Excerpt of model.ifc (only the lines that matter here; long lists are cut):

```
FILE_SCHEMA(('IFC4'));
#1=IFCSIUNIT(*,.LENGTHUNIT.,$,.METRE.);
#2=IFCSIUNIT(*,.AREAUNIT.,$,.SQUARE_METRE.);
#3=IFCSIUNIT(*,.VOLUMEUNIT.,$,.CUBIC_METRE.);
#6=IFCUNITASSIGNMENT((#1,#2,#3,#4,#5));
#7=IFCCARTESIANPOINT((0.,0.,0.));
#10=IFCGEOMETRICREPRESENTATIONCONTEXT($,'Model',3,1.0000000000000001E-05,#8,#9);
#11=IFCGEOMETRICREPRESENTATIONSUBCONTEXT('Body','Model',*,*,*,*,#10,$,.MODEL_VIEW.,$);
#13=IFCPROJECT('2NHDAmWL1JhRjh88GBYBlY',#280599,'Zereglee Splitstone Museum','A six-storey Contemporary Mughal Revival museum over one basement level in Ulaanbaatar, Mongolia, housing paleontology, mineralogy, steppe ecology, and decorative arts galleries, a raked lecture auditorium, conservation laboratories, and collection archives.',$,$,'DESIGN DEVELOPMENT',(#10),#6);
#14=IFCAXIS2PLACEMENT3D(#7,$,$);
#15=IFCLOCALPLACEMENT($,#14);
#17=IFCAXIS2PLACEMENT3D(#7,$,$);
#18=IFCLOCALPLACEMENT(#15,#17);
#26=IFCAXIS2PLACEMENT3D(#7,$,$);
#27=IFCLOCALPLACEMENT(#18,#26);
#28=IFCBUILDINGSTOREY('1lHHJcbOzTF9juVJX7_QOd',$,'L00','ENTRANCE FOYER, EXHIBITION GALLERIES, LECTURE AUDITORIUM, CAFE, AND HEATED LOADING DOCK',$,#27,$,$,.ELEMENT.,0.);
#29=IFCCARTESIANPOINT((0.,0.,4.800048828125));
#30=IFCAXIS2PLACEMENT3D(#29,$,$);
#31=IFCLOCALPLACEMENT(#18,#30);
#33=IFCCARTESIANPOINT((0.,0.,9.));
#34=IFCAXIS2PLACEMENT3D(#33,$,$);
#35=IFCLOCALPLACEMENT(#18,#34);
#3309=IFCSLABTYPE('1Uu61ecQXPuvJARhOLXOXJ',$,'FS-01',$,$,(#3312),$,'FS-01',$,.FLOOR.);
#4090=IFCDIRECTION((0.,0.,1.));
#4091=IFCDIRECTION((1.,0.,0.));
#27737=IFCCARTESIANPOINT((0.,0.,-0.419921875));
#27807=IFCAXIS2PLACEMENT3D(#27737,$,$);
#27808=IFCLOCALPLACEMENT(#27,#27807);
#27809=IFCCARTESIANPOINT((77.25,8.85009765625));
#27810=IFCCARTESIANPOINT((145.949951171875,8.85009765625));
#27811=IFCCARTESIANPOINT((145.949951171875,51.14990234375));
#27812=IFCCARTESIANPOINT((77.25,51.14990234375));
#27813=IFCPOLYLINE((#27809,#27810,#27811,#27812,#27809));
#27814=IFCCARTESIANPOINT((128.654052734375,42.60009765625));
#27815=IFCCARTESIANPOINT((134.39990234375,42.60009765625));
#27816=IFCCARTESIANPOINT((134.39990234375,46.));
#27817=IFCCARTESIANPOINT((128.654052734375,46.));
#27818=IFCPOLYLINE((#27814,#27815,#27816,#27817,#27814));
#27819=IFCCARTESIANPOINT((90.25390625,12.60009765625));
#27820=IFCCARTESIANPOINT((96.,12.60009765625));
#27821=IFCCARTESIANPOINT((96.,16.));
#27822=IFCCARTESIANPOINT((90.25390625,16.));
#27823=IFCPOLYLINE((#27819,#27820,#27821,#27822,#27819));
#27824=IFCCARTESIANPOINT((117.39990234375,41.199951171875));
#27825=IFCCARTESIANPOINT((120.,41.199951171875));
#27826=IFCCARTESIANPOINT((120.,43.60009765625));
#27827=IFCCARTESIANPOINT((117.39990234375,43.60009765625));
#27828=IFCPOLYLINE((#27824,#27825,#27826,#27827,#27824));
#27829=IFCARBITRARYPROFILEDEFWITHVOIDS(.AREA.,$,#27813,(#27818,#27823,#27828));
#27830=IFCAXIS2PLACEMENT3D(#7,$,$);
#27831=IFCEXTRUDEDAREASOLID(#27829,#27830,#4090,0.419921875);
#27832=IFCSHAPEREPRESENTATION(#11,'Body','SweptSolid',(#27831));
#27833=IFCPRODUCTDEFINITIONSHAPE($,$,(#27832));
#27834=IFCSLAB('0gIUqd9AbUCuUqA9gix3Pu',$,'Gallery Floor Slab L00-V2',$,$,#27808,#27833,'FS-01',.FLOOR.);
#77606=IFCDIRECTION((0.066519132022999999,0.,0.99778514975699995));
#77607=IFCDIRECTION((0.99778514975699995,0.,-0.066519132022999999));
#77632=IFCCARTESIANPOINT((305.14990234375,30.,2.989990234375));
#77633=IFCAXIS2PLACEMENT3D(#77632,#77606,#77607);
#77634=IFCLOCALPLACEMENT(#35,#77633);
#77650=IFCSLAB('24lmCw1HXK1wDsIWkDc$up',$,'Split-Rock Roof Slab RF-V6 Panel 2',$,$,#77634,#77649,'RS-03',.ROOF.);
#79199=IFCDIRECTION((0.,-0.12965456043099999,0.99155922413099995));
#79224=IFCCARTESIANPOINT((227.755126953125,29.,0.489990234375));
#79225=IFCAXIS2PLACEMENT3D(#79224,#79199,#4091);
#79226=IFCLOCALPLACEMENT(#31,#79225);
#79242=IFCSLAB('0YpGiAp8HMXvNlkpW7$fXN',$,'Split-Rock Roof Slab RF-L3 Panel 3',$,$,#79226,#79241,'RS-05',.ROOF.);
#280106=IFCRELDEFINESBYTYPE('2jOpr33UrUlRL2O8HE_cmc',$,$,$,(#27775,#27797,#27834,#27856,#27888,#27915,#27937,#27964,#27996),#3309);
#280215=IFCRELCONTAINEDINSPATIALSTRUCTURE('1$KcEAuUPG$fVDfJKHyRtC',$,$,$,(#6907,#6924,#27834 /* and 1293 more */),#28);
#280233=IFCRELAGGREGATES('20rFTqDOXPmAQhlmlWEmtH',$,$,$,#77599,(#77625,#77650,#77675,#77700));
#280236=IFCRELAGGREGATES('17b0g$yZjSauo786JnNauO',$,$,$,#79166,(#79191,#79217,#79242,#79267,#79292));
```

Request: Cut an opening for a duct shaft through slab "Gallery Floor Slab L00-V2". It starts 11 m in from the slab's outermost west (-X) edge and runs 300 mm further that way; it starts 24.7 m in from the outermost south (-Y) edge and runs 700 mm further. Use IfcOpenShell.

```python
import numpy as np
import ifcopenshell
import ifcopenshell.api.feature
import ifcopenshell.api.geometry
import ifcopenshell.api.root
import ifcopenshell.geom
import ifcopenshell.util.placement
import ifcopenshell.util.representation
import ifcopenshell.util.shape
import ifcopenshell.util.unit

model = ifcopenshell.open("model.ifc")
unit_scale = ifcopenshell.util.unit.calculate_unit_scale(model)
settings = ifcopenshell.geom.settings()


def volume(element):
    """Net volume in cubic metres, openings subtracted."""
    shape = ifcopenshell.geom.create_shape(settings, element)
    return ifcopenshell.util.shape.get_volume(shape.geometry)


slab = model.by_guid("0gIUqd9AbUCuUqA9gix3Pu")
before = volume(slab)

# Extent in the slab's own axes, in metres. The edges named are its -X and -Y sides.
slab_shape = ifcopenshell.geom.create_shape(settings, slab)
vertices = ifcopenshell.util.shape.get_vertices(slab_shape.geometry)
x_min, y_min, bottom = vertices.min(axis=0)
top = vertices[:, 2].max()

opening = ifcopenshell.api.root.create_entity(model, ifc_class="IfcOpeningElement", name="Duct shaft opening", predefined_type="OPENING")
context = ifcopenshell.util.representation.get_context(model, "Model", "Body", "MODEL_VIEW")
width, depth = 0.3, 0.7
outline = [(0.0, 0.0), (width, 0.0), (width, depth), (0.0, depth), (0.0, 0.0)]
# Overshoot both faces by 50 mm so the cut is clean.
shape = ifcopenshell.api.geometry.add_slab_representation(
    model, context=context, depth=top - bottom + 0.1, polyline=outline
)
ifcopenshell.api.geometry.assign_representation(model, product=opening, representation=shape)

matrix = ifcopenshell.util.placement.get_local_placement(slab.ObjectPlacement)
matrix[:, 3] = matrix @ np.append(np.array([x_min + 11, y_min + 24.7, bottom - 0.05]) / unit_scale, 1.0)
ifcopenshell.api.geometry.edit_object_placement(model, product=opening, matrix=matrix, is_si=False)
ifcopenshell.api.feature.add_feature(model, feature=opening, element=slab)

after = volume(slab)

print(f"slab volume {before:.3f} -> {after:.3f} m3")

model.write("model-out.ifc")
```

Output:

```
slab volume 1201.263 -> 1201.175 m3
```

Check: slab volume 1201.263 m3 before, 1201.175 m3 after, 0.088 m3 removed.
